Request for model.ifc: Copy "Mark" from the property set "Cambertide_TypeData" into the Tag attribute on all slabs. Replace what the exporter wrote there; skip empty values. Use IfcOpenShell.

First a look at what the model holds.

```python
import ifcopenshell
import ifcopenshell.util.element

model = ifcopenshell.open("model.ifc")
print(model.schema)
slabs = model.by_type("IfcSlab")
print(len(slabs), "slabs")
for e in slabs[:8]:
    source = ifcopenshell.util.element.get_pset(e, "Cambertide_TypeData", "Mark")
    target = e.Tag
    print(e.id(), repr(source), repr(target), sep=" | ")
```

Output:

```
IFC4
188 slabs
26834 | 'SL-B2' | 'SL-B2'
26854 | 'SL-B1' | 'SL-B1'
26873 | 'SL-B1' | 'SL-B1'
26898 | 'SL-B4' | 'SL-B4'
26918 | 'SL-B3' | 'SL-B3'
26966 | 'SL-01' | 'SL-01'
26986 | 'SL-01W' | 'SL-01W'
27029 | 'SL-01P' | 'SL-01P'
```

```python
import ifcopenshell
import ifcopenshell.util.element

model = ifcopenshell.open("model.ifc")

count = 0
for e in model.by_type("IfcSlab"):
    value = ifcopenshell.util.element.get_pset(e, "Cambertide_TypeData", "Mark")
    current = e.Tag
    if not value or not value.strip() or current == value:
        continue
    e.Tag = value
    count += 1

print(count, "slabs updated")

model.write("model_v2.ifc")
```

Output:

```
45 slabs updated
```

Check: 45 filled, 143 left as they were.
